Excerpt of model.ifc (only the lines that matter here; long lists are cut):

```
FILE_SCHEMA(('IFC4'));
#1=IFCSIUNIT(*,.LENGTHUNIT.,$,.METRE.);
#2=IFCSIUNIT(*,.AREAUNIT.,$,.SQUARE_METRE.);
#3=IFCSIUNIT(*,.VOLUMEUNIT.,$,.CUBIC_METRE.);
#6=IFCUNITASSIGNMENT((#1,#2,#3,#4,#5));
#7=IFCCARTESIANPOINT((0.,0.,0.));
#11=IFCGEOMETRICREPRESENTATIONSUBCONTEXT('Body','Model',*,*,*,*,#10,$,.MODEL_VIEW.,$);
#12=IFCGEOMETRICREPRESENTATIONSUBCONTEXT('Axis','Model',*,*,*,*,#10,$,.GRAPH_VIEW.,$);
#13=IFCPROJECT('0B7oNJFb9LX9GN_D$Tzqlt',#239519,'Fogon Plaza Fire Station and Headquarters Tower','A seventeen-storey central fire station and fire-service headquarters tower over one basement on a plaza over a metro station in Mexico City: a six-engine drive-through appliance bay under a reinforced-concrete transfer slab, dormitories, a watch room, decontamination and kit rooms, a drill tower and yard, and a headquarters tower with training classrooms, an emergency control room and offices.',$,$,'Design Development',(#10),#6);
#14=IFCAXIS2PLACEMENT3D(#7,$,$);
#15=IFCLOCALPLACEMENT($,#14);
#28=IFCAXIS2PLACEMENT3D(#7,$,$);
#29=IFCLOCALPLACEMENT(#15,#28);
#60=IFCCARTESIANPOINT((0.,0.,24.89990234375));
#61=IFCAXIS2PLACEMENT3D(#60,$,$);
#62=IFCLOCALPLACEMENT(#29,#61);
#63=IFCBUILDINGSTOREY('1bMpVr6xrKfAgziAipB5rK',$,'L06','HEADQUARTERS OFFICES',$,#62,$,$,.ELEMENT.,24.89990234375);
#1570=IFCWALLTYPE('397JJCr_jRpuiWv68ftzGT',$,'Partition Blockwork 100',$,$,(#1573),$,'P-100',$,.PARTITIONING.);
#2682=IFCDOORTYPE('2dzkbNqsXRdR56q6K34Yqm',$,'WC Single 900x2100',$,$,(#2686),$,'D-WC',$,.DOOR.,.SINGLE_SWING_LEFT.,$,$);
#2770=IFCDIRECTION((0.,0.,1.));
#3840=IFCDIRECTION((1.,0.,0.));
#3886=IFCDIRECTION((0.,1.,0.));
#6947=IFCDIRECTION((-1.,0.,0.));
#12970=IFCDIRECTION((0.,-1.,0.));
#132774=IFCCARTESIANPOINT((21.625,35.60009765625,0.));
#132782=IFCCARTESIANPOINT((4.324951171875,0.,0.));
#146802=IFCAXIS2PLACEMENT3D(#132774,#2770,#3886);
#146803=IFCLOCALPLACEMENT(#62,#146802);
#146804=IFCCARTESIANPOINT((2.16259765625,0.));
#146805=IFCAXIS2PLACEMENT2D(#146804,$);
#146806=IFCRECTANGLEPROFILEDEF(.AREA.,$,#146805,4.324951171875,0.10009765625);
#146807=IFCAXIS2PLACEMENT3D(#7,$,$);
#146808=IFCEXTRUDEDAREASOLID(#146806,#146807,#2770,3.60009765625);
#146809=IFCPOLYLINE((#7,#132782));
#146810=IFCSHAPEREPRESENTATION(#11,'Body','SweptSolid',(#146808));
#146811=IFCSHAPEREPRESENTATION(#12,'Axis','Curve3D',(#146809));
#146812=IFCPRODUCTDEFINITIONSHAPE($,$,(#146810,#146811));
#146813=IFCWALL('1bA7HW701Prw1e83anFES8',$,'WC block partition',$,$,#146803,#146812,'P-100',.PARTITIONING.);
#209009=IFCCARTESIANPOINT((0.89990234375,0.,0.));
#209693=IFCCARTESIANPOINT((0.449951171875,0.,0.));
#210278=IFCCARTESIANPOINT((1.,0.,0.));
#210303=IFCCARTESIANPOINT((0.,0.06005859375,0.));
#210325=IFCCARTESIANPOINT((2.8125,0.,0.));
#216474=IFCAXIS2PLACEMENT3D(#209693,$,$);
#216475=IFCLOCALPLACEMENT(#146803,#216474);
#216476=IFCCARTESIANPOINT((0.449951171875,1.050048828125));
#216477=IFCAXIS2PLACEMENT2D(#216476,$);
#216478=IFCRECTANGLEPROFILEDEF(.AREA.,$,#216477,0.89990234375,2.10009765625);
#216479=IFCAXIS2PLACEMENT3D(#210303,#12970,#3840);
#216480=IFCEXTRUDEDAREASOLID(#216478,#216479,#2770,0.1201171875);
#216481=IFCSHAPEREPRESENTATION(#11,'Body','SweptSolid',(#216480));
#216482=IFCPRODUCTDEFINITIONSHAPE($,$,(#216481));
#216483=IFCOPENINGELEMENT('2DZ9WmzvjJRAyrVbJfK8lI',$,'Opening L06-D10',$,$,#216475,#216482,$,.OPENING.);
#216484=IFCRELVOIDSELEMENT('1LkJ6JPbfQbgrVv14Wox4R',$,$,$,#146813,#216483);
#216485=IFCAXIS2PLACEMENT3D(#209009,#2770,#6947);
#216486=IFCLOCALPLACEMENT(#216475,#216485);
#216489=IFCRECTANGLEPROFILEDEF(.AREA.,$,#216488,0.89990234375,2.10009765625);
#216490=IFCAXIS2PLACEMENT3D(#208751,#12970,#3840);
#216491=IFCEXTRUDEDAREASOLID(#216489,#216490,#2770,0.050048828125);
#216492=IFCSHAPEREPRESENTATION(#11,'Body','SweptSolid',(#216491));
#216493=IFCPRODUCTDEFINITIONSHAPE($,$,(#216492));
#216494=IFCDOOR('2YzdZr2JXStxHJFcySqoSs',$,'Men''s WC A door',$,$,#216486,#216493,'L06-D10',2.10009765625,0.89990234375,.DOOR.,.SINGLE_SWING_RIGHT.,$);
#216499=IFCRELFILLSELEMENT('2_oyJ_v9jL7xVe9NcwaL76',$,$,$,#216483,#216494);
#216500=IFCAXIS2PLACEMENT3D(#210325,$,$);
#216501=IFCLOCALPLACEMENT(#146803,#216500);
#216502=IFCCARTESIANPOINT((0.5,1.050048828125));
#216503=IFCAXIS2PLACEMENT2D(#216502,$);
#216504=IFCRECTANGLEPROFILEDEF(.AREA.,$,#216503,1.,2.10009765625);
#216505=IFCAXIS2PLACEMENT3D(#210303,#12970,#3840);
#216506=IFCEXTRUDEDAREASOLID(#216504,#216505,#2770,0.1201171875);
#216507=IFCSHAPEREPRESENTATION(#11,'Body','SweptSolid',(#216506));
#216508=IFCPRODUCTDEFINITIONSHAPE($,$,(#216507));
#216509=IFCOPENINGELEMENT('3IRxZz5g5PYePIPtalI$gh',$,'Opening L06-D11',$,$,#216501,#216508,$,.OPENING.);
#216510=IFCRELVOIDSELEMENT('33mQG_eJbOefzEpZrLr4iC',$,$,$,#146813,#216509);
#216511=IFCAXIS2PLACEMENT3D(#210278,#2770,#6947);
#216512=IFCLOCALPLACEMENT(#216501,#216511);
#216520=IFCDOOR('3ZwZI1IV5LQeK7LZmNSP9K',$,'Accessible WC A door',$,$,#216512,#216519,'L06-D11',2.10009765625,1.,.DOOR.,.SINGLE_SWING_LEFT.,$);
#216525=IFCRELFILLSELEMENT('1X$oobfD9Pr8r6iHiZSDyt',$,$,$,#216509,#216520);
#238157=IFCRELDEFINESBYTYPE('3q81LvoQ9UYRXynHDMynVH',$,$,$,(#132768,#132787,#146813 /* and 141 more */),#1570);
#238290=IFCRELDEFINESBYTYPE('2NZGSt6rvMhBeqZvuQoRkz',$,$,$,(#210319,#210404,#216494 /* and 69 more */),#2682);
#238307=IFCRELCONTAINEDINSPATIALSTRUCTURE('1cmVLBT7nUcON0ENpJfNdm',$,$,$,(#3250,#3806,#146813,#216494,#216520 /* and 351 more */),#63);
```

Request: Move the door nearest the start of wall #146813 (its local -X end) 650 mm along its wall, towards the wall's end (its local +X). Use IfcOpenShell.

```python
import ifcopenshell
import ifcopenshell.api.geometry
import ifcopenshell.util.placement
import ifcopenshell.util.unit

model = ifcopenshell.open("model.ifc")
unit_scale = ifcopenshell.util.unit.calculate_unit_scale(model)

door = model.by_id(216494)
opening = door.FillsVoids[0].RelatingOpeningElement
wall = opening.VoidsElements[0].RelatingBuildingElement

wall_matrix = ifcopenshell.util.placement.get_local_placement(wall.ObjectPlacement)
shift = wall_matrix[:3, 0] * 0.65 / unit_scale
before = ifcopenshell.util.placement.get_local_placement(door.ObjectPlacement)[:3, 3].copy()

# The door is placed relative to its opening, so it follows when the opening moves.
matrix = ifcopenshell.util.placement.get_local_placement(opening.ObjectPlacement)
matrix[:3, 3] += shift
ifcopenshell.api.geometry.edit_object_placement(
    model, product=opening, matrix=matrix, is_si=False, should_transform_children=True
)

after = ifcopenshell.util.placement.get_local_placement(door.ObjectPlacement)[:3, 3]
print("door moved by", (after - before).round(3) + 0.0)

model.write("model-out.ifc")
```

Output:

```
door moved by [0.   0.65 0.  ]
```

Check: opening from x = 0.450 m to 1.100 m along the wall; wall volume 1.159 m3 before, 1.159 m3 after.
